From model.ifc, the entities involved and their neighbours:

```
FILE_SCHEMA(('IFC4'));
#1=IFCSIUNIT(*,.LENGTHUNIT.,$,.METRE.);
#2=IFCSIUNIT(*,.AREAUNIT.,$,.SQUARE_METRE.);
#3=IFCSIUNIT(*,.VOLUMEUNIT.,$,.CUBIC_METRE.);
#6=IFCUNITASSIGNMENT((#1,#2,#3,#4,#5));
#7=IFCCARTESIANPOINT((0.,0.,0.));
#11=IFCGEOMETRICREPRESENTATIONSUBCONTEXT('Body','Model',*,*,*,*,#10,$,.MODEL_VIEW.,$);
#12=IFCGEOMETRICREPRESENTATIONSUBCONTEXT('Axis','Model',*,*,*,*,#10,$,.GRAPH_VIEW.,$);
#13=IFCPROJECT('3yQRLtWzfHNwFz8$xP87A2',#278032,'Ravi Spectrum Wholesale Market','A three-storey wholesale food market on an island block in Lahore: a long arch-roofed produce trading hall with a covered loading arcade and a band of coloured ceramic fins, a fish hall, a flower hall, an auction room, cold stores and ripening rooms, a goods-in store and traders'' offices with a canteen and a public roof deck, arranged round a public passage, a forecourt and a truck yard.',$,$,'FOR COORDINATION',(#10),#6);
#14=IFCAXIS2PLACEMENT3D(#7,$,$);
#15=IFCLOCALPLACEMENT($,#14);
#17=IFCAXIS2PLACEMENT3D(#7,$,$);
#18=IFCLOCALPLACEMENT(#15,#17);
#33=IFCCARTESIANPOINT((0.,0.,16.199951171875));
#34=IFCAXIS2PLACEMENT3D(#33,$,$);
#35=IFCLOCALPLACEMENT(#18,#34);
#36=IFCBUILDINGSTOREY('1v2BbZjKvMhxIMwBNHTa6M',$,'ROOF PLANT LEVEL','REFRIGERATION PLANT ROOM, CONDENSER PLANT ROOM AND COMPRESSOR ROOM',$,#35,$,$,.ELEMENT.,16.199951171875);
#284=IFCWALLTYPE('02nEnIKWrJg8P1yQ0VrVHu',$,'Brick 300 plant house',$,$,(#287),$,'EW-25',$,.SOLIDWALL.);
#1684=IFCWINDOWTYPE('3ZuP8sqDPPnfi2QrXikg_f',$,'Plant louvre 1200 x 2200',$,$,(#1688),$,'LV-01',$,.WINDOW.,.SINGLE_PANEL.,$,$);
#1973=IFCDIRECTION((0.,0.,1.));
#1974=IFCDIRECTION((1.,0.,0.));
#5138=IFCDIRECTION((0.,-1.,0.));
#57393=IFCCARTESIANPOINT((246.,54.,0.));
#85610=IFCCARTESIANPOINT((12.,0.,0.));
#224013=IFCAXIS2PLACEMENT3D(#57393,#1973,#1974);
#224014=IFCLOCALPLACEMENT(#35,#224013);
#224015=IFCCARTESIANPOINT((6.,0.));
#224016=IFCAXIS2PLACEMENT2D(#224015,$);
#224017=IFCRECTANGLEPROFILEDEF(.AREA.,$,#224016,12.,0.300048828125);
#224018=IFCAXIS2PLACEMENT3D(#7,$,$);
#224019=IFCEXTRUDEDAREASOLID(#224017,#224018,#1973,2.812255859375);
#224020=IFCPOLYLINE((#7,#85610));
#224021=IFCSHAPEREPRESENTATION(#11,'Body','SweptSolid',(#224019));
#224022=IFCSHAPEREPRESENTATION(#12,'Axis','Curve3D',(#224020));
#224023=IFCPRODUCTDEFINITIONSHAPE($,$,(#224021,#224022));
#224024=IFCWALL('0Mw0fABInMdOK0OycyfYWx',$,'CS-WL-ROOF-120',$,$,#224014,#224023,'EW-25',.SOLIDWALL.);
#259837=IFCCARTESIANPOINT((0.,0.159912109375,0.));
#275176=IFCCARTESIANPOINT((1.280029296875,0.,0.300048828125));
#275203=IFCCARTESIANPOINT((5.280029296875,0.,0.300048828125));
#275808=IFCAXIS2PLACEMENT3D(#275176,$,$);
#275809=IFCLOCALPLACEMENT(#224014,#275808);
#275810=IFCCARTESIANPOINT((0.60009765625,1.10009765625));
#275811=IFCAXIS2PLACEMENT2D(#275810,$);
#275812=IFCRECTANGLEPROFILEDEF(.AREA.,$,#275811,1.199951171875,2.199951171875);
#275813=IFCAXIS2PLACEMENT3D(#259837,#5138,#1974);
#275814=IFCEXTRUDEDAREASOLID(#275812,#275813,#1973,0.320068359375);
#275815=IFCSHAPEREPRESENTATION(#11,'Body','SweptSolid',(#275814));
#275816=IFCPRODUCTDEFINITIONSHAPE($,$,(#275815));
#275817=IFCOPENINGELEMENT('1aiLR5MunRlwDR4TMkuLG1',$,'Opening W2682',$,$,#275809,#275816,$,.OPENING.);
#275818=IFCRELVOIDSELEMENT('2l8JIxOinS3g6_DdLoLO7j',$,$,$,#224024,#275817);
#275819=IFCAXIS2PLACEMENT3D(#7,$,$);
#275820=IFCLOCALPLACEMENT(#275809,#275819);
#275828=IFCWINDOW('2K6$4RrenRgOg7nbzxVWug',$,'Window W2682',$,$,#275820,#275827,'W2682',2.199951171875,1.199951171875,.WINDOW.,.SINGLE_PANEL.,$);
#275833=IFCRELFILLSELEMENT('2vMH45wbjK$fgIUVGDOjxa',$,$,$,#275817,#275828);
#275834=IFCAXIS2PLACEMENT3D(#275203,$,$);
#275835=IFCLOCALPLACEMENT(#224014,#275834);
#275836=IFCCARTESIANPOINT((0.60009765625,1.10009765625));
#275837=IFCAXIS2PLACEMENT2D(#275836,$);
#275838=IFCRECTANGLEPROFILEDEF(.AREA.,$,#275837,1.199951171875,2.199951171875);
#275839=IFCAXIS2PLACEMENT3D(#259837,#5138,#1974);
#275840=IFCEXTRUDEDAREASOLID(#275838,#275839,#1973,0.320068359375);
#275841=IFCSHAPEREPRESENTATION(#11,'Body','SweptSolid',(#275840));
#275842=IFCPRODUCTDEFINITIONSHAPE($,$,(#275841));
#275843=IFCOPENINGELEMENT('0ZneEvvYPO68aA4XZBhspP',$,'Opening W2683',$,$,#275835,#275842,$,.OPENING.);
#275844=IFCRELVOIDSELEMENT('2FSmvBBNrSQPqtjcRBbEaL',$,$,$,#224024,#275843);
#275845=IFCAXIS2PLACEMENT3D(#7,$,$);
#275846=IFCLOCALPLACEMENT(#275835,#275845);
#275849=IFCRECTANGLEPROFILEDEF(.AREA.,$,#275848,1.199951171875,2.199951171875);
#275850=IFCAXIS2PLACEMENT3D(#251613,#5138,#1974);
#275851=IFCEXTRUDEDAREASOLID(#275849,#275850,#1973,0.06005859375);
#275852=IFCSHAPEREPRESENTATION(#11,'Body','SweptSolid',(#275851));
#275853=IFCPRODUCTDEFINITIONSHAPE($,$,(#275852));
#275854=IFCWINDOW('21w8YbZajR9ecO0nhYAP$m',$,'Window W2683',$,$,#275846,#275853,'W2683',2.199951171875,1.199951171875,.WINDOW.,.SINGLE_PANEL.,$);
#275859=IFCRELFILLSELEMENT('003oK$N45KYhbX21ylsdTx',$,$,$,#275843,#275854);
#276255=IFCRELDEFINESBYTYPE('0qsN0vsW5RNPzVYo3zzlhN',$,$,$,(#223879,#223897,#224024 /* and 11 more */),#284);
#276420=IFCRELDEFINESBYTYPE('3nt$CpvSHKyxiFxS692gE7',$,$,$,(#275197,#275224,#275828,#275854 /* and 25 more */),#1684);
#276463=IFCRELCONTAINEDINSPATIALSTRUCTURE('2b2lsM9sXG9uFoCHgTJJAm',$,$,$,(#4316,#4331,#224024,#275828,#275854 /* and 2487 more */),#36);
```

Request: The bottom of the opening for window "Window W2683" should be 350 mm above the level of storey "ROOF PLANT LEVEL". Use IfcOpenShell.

```python
import numpy as np
import ifcopenshell
import ifcopenshell.api.geometry
import ifcopenshell.geom
import ifcopenshell.util.element
import ifcopenshell.util.placement
import ifcopenshell.util.shape
import ifcopenshell.util.unit

model = ifcopenshell.open("model.ifc")
unit_scale = ifcopenshell.util.unit.calculate_unit_scale(model)

window = model.by_id(275854)
opening = window.FillsVoids[0].RelatingOpeningElement
storey = ifcopenshell.util.element.get_container(window, ifc_class="IfcBuildingStorey")
level = ifcopenshell.util.placement.get_local_placement(storey.ObjectPlacement)[2, 3]

# The opening's origin need not be at the sill, so measure its lowest point.
shape = ifcopenshell.geom.create_shape(ifcopenshell.geom.settings(), opening)
bottom = ifcopenshell.util.shape.get_shape_bottom_elevation(shape, shape.geometry) / unit_scale
dz = level + 0.35 / unit_scale - bottom

shift = np.array([0.0, 0.0, dz])
# The window is placed relative to its opening, so it follows when the opening moves.
matrix = ifcopenshell.util.placement.get_local_placement(opening.ObjectPlacement)
matrix[:3, 3] += shift
ifcopenshell.api.geometry.edit_object_placement(
    model, product=opening, matrix=matrix, is_si=False, should_transform_children=True
)

print(f"moved by {dz * unit_scale:+.3f} m")

model.write("model_edited.ifc")
```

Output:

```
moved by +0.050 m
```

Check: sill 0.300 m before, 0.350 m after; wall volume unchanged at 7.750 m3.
